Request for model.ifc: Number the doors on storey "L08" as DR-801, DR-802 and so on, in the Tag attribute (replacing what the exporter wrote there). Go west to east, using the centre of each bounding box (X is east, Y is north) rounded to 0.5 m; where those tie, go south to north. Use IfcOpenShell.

First a look at what the model holds.

```python
import ifcopenshell
import ifcopenshell.util.element
import ifcopenshell.util.placement

model = ifcopenshell.open("model.ifc")
print(model.schema)
storey = next(s for s in model.by_type("IfcBuildingStorey") if s.Name == "L08")
doors = [e for e in ifcopenshell.util.element.get_decomposition(storey) if e.is_a("IfcDoor")]
for e in sorted(doors, key=lambda e: e.id()):
    origin = ifcopenshell.util.placement.get_local_placement(e.ObjectPlacement)[:3, 3]
    print(e.id(), e.Tag, e.Name, origin.round(2) + 0.0, sep=" | ")
```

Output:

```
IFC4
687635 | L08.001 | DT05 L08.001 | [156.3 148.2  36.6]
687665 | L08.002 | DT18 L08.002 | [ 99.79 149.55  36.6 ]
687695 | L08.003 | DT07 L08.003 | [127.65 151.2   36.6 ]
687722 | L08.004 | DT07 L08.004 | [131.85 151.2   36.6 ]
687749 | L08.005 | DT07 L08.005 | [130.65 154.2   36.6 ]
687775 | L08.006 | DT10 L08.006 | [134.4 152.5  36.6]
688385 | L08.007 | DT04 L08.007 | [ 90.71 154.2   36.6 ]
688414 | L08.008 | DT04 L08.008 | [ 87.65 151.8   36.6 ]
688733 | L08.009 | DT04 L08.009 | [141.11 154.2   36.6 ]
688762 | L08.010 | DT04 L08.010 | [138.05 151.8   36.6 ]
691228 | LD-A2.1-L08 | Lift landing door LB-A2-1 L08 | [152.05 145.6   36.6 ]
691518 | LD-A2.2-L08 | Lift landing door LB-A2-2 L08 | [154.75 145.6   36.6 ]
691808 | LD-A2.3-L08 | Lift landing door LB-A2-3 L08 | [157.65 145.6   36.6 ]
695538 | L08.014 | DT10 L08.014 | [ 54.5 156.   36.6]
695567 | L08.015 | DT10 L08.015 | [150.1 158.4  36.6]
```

```python
import ifcopenshell
import ifcopenshell.geom
import ifcopenshell.util.element
import ifcopenshell.util.shape

model = ifcopenshell.open("model.ifc")
settings = ifcopenshell.geom.settings()
settings.set("use-world-coords", True)


def centre(element):
    shape = ifcopenshell.geom.create_shape(settings, element)
    return ifcopenshell.util.shape.get_bbox_centroid(shape.geometry)


storey = next(s for s in model.by_type("IfcBuildingStorey") if s.Name == "L08")
doors = [e for e in ifcopenshell.util.element.get_decomposition(storey) if e.is_a("IfcDoor")]

# Insertion points can sit at a corner or the storey origin, so sort by the geometry (in metres).
centres = {e: centre(e) for e in doors}
doors.sort(key=lambda e: (round(centres[e][0] / 0.5), centres[e][1]))

for i, e in enumerate(doors, start=1):
    number = f"DR-8{i:02d}"
    e.Tag = number
    print(e.id(), number)

model.write("model_rev.ifc")
```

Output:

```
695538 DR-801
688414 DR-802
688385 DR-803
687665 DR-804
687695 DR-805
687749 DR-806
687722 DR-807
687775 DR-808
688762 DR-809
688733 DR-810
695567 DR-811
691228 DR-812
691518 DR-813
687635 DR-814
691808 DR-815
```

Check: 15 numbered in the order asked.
